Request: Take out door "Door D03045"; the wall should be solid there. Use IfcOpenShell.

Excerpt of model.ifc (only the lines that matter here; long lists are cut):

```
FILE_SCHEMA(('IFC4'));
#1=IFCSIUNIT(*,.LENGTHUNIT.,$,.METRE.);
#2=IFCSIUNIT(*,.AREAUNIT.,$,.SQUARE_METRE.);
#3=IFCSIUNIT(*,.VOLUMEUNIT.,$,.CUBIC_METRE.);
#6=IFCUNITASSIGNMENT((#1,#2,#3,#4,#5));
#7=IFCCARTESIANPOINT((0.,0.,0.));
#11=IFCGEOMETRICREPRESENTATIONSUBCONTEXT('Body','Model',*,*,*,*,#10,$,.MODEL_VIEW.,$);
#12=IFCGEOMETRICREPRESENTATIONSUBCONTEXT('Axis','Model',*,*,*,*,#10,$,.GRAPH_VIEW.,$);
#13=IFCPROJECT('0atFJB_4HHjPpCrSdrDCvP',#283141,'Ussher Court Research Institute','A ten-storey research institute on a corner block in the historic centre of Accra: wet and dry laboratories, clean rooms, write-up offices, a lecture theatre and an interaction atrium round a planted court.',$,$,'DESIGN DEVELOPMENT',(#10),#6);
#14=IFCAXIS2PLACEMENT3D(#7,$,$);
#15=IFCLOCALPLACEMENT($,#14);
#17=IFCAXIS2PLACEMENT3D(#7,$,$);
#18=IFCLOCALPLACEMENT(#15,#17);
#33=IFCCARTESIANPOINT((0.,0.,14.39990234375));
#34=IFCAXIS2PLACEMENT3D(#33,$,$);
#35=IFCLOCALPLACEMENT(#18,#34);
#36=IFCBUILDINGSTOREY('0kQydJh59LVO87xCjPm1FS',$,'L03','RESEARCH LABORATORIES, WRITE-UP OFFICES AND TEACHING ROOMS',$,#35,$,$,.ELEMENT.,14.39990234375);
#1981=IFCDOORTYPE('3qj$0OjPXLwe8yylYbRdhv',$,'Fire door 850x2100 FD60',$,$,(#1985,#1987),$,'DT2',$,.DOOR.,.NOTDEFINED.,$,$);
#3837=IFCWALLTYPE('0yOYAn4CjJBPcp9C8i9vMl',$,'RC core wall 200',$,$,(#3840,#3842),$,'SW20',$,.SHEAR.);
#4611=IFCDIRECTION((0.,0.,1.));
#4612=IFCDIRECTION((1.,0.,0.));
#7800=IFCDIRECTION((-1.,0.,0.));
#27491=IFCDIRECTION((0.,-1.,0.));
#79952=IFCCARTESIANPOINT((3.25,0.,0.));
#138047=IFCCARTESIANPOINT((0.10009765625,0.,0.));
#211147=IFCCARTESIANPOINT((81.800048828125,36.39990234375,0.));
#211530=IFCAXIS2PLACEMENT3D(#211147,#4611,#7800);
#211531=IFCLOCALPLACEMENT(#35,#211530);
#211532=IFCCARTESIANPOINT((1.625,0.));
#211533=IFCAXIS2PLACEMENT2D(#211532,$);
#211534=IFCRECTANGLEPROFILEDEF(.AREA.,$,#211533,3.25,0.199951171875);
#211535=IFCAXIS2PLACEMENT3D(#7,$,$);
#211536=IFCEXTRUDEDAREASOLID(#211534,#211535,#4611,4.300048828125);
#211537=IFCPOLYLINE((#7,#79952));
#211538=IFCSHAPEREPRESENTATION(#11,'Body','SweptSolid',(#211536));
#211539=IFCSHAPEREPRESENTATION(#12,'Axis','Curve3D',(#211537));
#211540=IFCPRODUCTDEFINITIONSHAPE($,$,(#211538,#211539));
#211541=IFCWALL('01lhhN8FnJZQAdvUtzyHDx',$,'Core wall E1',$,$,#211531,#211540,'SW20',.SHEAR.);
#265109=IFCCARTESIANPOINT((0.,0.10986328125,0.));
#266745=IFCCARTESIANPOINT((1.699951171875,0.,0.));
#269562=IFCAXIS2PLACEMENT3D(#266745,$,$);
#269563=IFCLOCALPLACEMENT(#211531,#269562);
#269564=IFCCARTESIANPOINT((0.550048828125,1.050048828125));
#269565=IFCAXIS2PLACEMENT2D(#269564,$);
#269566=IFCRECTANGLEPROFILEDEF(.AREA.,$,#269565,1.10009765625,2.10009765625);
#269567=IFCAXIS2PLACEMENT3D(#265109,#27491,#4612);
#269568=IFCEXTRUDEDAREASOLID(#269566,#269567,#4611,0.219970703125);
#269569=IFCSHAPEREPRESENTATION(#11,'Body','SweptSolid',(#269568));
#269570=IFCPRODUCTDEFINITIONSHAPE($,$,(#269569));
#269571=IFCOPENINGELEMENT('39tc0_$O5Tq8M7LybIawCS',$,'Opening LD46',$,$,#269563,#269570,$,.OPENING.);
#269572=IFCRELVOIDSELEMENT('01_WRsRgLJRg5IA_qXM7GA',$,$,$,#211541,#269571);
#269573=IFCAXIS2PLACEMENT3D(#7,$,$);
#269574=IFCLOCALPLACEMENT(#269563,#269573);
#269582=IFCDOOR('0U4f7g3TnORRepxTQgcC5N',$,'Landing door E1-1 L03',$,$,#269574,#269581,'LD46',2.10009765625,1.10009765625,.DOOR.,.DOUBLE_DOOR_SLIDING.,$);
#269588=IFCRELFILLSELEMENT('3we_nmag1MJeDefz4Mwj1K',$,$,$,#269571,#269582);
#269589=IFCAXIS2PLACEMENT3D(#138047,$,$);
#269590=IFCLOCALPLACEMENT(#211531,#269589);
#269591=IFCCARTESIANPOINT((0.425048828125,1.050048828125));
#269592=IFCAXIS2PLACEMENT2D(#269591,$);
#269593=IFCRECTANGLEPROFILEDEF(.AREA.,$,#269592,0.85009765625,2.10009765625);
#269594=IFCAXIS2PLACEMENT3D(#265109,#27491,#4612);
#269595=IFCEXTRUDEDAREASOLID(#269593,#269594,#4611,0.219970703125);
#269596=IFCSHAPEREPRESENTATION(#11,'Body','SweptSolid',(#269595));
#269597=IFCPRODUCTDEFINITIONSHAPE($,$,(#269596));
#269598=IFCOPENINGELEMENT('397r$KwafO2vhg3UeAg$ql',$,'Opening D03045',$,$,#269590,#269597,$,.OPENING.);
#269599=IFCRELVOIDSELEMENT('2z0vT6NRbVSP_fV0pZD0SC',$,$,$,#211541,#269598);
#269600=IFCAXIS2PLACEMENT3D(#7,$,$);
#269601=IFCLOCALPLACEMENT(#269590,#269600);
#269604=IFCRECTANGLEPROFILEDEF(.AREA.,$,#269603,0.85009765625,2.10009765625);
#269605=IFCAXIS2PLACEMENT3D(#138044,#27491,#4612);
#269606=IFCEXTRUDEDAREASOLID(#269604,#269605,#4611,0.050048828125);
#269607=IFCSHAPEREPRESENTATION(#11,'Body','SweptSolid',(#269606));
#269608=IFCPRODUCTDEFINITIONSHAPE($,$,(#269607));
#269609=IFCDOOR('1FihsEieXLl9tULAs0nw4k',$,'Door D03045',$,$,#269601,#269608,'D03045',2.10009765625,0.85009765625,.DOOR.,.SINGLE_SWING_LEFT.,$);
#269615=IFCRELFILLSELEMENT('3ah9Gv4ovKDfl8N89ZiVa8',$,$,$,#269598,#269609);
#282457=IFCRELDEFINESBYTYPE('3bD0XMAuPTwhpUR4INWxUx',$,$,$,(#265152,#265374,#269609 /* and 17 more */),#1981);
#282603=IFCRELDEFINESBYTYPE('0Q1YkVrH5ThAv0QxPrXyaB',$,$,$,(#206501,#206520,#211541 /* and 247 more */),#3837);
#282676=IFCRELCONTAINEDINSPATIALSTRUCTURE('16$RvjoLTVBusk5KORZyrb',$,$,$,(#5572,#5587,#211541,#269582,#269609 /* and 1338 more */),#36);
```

```python
import ifcopenshell
import ifcopenshell.api.feature
import ifcopenshell.api.root
import ifcopenshell.geom
import ifcopenshell.util.shape

model = ifcopenshell.open("model.ifc")
settings = ifcopenshell.geom.settings()


def volume(element):
    """Net volume in cubic metres, openings subtracted."""
    shape = ifcopenshell.geom.create_shape(settings, element)
    return ifcopenshell.util.shape.get_volume(shape.geometry)


door = model.by_id(269609)
opening = door.FillsVoids[0].RelatingOpeningElement
wall = opening.VoidsElements[0].RelatingBuildingElement
before = volume(wall)

ifcopenshell.api.root.remove_product(model, product=door)
ifcopenshell.api.feature.remove_feature(model, feature=opening)

after = volume(wall)

print(f"wall volume {before:.3f} -> {after:.3f} m3")

model.write("model_v2.ifc")
```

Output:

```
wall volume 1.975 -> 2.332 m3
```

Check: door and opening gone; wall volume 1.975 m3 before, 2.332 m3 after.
